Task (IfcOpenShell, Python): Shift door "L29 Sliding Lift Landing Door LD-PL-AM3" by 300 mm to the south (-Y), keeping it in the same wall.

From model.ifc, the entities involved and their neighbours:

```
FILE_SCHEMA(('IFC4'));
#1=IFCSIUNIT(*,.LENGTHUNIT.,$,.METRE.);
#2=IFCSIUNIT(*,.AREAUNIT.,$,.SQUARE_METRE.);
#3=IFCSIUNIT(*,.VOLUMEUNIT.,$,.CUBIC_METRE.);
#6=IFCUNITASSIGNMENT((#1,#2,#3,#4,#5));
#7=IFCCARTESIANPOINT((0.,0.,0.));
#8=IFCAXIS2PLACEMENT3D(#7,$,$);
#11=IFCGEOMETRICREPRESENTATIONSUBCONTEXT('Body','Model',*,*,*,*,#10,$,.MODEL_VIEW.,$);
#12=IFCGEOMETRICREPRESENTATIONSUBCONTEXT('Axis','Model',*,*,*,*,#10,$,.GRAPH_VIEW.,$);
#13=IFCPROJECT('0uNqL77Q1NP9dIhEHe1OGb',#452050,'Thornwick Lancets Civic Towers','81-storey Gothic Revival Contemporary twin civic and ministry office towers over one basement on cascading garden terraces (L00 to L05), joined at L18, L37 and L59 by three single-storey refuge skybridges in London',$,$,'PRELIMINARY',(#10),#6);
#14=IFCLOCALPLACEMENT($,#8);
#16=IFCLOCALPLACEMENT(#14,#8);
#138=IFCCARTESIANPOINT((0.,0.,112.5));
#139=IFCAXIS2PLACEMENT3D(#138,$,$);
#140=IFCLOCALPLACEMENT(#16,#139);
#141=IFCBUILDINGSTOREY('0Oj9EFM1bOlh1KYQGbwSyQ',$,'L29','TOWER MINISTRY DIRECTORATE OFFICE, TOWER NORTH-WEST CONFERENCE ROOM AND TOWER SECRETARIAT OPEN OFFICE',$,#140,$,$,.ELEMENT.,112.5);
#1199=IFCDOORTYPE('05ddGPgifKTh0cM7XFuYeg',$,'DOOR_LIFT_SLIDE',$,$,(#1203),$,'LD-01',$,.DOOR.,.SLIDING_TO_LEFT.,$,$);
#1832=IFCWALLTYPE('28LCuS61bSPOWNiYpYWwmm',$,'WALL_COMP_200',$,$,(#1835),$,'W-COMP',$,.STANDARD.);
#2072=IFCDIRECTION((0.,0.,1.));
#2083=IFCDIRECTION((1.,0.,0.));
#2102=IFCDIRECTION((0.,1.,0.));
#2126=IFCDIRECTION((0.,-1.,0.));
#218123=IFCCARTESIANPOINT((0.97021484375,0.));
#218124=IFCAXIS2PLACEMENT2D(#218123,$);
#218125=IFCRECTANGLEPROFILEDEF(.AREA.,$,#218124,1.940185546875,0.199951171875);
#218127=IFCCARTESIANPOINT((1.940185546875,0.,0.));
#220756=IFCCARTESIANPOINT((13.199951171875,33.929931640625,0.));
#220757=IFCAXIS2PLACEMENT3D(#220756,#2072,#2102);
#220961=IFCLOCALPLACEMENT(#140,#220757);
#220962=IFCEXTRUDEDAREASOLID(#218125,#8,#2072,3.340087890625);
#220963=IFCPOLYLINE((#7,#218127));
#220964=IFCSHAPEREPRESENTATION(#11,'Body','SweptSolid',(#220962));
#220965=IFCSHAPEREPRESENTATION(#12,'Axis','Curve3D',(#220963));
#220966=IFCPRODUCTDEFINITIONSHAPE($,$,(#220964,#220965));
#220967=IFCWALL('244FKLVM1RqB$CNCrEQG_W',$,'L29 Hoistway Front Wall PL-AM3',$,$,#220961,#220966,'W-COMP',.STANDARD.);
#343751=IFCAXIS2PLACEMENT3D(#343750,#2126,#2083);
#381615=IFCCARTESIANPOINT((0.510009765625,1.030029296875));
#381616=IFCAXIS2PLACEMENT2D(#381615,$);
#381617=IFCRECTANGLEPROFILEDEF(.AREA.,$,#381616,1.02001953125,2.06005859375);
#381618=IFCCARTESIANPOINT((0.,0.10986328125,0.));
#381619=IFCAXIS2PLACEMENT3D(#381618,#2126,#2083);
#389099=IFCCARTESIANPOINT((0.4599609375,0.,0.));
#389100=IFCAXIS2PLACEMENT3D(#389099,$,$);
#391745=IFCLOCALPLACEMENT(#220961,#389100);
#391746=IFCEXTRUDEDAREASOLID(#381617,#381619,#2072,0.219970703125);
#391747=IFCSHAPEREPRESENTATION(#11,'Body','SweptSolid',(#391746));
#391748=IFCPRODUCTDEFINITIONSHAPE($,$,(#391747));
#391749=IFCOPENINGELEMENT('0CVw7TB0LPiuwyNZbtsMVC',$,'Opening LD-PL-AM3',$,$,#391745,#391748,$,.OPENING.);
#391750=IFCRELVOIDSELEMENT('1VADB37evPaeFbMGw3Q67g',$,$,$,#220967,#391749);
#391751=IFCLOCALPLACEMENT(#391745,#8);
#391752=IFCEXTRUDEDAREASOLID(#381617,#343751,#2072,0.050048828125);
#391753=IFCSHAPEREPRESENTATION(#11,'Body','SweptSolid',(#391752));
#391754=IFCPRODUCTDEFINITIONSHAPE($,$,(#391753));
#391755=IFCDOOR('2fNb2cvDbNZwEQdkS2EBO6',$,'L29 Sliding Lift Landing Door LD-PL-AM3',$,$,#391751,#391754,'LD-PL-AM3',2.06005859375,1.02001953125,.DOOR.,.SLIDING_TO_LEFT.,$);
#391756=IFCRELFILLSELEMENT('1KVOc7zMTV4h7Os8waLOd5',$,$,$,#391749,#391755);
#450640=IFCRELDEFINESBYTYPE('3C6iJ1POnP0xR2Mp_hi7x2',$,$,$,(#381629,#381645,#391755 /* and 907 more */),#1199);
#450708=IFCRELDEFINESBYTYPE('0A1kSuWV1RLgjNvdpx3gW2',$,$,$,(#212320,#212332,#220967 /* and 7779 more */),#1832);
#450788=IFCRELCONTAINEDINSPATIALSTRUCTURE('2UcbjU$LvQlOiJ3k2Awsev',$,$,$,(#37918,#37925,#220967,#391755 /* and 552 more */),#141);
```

```python
import ifcopenshell
import ifcopenshell.api.geometry
import ifcopenshell.util.placement
import ifcopenshell.util.unit

model = ifcopenshell.open("model.ifc")
unit_scale = ifcopenshell.util.unit.calculate_unit_scale(model)

door = model.by_guid("2fNb2cvDbNZwEQdkS2EBO6")
opening = door.FillsVoids[0].RelatingOpeningElement
wall = opening.VoidsElements[0].RelatingBuildingElement

wall_matrix = ifcopenshell.util.placement.get_local_placement(wall.ObjectPlacement)
shift = wall_matrix[:3, 0] * -0.3 / unit_scale
before = ifcopenshell.util.placement.get_local_placement(door.ObjectPlacement)[:3, 3].copy()

# The door is placed relative to its opening, so it follows when the opening moves.
matrix = ifcopenshell.util.placement.get_local_placement(opening.ObjectPlacement)
matrix[:3, 3] += shift
ifcopenshell.api.geometry.edit_object_placement(
    model, product=opening, matrix=matrix, is_si=False, should_transform_children=True
)

after = ifcopenshell.util.placement.get_local_placement(door.ObjectPlacement)[:3, 3]
print("door moved by", (after - before).round(3) + 0.0)

model.write("model_rev.ifc")
```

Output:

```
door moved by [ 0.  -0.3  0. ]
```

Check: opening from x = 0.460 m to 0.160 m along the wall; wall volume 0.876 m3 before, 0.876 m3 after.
